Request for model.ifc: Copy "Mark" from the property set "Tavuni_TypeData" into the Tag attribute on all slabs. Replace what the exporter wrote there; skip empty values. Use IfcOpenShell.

First a look at what the model holds.

```python
import ifcopenshell
import ifcopenshell.util.element

model = ifcopenshell.open("model.ifc")
print(model.schema)
slabs = model.by_type("IfcSlab")
print(len(slabs), "slabs")
for e in slabs[:8]:
    source = ifcopenshell.util.element.get_pset(e, "Tavuni_TypeData", "Mark")
    target = e.Tag
    print(e.id(), repr(source), repr(target), sep=" | ")
```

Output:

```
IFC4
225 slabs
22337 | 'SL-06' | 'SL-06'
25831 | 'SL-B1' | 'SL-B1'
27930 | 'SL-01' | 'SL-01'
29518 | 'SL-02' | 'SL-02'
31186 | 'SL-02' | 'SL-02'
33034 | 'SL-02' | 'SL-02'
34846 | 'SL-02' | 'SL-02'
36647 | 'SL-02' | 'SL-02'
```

```python
import ifcopenshell
import ifcopenshell.util.element

model = ifcopenshell.open("model.ifc")

count = 0
for e in model.by_type("IfcSlab"):
    value = ifcopenshell.util.element.get_pset(e, "Tavuni_TypeData", "Mark")
    current = e.Tag
    if not value or not value.strip() or current == value:
        continue
    e.Tag = value
    count += 1

print(count, "slabs updated")

model.write("model_v2.ifc")
```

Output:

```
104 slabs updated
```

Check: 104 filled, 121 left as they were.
